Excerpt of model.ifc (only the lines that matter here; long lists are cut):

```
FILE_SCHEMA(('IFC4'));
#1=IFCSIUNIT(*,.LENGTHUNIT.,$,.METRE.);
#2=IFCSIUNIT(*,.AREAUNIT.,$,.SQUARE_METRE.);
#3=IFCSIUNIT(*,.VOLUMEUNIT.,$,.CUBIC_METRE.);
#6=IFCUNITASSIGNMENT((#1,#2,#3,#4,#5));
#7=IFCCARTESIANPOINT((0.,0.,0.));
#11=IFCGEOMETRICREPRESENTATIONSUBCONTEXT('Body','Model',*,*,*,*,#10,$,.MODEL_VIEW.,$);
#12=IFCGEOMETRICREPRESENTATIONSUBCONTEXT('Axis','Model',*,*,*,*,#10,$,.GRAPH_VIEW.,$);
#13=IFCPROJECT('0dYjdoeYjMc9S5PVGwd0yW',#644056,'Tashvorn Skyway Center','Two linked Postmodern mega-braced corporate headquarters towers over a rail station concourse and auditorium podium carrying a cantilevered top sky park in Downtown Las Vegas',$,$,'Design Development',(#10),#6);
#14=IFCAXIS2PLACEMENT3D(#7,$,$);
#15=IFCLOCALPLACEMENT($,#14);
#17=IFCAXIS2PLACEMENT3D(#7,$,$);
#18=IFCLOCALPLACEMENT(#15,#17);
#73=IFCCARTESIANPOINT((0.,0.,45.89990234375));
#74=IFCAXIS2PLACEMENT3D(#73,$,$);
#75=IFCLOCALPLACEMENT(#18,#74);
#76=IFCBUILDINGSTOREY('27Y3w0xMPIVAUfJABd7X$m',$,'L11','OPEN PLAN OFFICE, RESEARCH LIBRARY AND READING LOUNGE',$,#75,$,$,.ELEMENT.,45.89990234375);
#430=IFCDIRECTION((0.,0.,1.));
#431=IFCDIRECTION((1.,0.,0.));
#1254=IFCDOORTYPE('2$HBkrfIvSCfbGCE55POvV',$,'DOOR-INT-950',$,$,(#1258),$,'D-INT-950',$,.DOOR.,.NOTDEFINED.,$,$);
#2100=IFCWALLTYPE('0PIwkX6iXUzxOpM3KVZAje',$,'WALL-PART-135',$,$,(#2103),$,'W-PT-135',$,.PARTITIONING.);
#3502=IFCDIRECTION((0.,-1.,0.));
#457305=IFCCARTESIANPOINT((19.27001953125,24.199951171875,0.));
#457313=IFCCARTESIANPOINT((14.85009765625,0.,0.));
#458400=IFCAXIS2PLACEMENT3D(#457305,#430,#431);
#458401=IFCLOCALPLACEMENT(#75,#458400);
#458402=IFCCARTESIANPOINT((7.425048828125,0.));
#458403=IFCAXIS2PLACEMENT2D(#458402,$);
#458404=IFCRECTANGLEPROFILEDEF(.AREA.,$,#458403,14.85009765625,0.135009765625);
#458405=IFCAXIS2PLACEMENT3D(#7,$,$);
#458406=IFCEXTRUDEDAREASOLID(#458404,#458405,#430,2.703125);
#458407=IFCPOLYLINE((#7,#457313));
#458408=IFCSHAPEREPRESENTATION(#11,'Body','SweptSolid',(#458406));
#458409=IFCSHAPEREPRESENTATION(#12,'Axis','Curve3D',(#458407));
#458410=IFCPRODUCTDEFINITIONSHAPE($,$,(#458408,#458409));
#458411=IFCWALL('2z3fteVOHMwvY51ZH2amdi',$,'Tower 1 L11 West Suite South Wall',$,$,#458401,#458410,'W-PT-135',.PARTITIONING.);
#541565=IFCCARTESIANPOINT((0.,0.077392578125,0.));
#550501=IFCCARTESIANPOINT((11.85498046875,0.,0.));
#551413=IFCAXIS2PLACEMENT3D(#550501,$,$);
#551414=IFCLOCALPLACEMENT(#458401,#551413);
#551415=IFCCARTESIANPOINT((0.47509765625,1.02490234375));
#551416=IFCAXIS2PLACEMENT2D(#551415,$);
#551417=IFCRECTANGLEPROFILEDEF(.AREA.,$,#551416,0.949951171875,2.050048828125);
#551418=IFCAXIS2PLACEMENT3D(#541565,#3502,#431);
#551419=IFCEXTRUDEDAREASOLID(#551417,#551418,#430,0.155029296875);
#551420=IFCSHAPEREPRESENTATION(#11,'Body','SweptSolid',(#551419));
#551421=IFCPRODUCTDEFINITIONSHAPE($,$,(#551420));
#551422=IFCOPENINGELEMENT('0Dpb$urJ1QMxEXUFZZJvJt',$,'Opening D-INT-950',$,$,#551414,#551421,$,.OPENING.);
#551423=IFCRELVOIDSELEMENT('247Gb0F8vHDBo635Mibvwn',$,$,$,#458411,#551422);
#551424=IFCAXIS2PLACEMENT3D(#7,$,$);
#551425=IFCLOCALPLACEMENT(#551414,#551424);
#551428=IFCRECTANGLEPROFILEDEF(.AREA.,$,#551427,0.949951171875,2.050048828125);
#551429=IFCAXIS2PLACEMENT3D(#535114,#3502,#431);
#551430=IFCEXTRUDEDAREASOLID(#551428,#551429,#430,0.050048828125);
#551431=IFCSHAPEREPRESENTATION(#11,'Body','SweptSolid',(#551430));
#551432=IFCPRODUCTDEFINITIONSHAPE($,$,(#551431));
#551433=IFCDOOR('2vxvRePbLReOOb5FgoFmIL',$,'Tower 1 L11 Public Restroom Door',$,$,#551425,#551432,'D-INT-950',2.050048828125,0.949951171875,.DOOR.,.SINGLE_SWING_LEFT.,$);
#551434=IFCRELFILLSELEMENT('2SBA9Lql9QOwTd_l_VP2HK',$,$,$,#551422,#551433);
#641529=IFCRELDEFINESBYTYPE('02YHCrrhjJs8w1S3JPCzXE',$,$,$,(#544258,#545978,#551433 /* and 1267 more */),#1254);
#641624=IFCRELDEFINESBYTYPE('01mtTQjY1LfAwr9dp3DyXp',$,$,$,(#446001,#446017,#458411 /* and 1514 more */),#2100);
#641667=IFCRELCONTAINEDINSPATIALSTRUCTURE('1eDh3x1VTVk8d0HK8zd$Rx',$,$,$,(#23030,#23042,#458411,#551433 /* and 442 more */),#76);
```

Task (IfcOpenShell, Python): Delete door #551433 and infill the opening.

```python
import ifcopenshell
import ifcopenshell.api.feature
import ifcopenshell.api.root
import ifcopenshell.geom
import ifcopenshell.util.shape

model = ifcopenshell.open("model.ifc")
settings = ifcopenshell.geom.settings()


def volume(element):
    """Net volume in cubic metres, openings subtracted."""
    shape = ifcopenshell.geom.create_shape(settings, element)
    return ifcopenshell.util.shape.get_volume(shape.geometry)


door = model.by_id(551433)
opening = door.FillsVoids[0].RelatingOpeningElement
wall = opening.VoidsElements[0].RelatingBuildingElement
before = volume(wall)

ifcopenshell.api.root.remove_product(model, product=door)
ifcopenshell.api.feature.remove_feature(model, feature=opening)

after = volume(wall)

print(f"wall volume {before:.3f} -> {after:.3f} m3")

model.write("model_updated.ifc")
```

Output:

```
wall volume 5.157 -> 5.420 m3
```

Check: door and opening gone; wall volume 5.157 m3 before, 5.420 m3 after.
